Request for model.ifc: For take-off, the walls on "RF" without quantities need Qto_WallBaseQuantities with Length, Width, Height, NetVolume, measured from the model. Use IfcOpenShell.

First a look at what the model holds.

```python
import ifcopenshell
import ifcopenshell.util.element
import ifcopenshell.util.unit

model = ifcopenshell.open("model.ifc")
print(model.schema)
for unit_type in ("LENGTHUNIT", "AREAUNIT", "VOLUMEUNIT"):
    print(unit_type, ifcopenshell.util.unit.calculate_unit_scale(model, unit_type))
storey = next(s for s in model.by_type("IfcBuildingStorey") if s.Name == "RF")
walls = [e for e in ifcopenshell.util.element.get_decomposition(storey) if e.is_a("IfcWall")]
for e in sorted(walls, key=lambda e: e.id()):
    print(e.id(), e.is_a(), e.Name, list(ifcopenshell.util.element.get_psets(e, qtos_only=True)), sep=" | ")
```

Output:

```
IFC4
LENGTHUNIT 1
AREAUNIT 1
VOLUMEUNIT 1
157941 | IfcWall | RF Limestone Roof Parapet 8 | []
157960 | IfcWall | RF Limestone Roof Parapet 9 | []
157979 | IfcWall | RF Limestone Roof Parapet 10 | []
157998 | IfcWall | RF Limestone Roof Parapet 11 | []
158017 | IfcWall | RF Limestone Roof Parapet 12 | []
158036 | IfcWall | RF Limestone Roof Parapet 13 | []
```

```python
import ifcopenshell
import ifcopenshell.api.pset
import ifcopenshell.geom
import ifcopenshell.util.element
import ifcopenshell.util.shape
import ifcopenshell.util.unit

model = ifcopenshell.open("model.ifc")
unit_scale = ifcopenshell.util.unit.calculate_unit_scale(model)
volume_scale = ifcopenshell.util.unit.calculate_unit_scale(model, "VOLUMEUNIT")
settings = ifcopenshell.geom.settings()

storey = next(s for s in model.by_type("IfcBuildingStorey") if s.Name == "RF")
walls = [e for e in ifcopenshell.util.element.get_decomposition(storey) if e.is_a("IfcWall")]

for e in sorted(walls, key=lambda e: e.id()):
    if ifcopenshell.util.element.get_psets(e, qtos_only=True, should_inherit=False):
        continue
    # Geometry comes back in metres, in the element's own axes.
    shape = ifcopenshell.geom.create_shape(settings, e)
    values = {
        "Length": ifcopenshell.util.shape.get_x(shape.geometry) / unit_scale,
        "Width": ifcopenshell.util.shape.get_y(shape.geometry) / unit_scale,
        "Height": ifcopenshell.util.shape.get_z(shape.geometry) / unit_scale,
        "NetVolume": ifcopenshell.util.shape.get_volume(shape.geometry) / volume_scale,
    }
    qto = ifcopenshell.api.pset.add_qto(model, product=e, name="Qto_WallBaseQuantities")
    ifcopenshell.api.pset.edit_qto(model, qto=qto, properties=values)
    print(e.id(), {k: round(v, 3) for k, v in values.items()})

model.write("model_rev.ifc")
```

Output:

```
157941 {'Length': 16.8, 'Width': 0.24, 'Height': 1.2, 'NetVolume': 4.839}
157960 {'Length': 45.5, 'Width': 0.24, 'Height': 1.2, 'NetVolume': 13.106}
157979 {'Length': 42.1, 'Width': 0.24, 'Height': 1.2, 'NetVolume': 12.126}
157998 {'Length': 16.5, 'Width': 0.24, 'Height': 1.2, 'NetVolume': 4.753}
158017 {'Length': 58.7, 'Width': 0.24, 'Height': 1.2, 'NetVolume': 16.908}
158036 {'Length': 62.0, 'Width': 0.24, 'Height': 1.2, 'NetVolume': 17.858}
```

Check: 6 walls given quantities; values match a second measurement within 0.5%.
